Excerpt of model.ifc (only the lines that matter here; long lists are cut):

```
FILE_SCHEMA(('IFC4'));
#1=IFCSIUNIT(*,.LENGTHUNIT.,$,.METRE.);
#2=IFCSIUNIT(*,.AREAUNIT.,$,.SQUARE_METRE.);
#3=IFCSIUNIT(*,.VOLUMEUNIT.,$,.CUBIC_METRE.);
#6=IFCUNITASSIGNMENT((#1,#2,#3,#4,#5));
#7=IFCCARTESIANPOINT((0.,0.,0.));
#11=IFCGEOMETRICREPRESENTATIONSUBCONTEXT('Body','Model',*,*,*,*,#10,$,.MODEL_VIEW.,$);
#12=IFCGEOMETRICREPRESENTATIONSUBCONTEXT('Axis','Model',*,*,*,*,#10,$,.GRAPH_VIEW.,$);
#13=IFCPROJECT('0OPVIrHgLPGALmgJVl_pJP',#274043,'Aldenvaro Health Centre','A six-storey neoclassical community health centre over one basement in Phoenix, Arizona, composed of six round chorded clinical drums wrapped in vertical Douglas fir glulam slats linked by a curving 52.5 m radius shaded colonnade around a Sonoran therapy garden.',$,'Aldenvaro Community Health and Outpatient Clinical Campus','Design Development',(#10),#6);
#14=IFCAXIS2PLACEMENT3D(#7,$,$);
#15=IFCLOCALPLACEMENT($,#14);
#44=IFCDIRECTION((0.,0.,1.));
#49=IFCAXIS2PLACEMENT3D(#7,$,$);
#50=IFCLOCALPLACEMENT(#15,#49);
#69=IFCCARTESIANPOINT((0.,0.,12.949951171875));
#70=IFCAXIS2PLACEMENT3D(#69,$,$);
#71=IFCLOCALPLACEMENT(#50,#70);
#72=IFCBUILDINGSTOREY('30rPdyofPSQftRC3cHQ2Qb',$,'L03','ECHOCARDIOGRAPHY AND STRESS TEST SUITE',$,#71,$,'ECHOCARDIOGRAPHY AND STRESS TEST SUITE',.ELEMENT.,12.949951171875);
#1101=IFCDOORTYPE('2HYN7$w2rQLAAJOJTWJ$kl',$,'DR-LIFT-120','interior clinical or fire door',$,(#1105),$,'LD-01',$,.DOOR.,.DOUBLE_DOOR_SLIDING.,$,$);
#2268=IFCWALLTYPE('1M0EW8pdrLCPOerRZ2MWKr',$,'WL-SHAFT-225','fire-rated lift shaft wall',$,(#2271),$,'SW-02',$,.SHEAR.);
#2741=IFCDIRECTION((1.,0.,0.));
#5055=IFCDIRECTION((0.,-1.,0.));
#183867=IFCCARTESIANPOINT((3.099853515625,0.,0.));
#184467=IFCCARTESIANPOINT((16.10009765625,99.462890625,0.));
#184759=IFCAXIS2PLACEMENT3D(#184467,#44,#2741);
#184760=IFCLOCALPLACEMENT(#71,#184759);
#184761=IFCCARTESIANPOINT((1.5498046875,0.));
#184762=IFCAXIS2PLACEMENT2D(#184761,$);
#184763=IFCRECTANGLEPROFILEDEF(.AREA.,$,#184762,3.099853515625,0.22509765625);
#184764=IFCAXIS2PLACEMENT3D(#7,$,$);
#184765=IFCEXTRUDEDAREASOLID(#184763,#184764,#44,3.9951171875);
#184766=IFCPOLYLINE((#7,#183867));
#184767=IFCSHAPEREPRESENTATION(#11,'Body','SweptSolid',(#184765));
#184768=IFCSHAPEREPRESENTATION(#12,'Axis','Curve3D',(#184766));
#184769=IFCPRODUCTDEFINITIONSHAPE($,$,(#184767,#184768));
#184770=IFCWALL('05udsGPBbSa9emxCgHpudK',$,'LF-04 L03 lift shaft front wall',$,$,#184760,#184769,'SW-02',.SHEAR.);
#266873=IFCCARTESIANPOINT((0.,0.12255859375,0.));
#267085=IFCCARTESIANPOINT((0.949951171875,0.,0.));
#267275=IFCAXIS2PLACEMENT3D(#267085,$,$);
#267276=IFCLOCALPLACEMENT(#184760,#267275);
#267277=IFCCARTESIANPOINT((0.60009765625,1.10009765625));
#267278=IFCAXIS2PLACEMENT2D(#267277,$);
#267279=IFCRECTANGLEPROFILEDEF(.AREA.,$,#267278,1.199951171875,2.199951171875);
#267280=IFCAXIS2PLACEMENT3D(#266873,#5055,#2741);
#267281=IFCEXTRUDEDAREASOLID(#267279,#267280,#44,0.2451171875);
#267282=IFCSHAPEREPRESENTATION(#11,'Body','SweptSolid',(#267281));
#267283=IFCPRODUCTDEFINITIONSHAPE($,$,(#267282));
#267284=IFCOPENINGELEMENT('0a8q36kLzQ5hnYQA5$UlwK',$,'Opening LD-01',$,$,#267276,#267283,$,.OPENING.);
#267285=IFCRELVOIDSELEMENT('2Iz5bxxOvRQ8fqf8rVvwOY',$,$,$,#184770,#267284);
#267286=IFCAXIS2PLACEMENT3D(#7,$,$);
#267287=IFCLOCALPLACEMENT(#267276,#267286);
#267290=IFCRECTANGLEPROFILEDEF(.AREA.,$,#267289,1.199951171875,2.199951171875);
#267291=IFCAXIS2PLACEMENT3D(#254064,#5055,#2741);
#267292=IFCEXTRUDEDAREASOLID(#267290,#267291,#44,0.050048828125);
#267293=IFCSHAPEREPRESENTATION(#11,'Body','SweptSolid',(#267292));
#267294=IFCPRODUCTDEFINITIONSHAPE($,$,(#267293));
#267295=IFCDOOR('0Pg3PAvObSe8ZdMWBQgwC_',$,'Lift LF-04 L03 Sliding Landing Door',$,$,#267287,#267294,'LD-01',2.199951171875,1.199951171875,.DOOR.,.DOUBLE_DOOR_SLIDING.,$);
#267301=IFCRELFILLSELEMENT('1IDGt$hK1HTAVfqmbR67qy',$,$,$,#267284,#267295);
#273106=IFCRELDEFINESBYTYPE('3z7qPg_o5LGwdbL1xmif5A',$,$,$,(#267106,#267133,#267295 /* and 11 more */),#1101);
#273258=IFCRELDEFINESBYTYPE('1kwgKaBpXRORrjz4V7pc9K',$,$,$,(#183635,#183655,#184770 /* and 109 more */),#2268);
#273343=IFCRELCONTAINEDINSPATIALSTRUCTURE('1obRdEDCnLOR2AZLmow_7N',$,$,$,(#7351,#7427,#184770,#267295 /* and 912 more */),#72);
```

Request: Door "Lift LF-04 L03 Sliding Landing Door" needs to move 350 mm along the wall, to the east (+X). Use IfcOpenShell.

```python
import ifcopenshell
import ifcopenshell.api.geometry
import ifcopenshell.util.placement
import ifcopenshell.util.unit

model = ifcopenshell.open("model.ifc")
unit_scale = ifcopenshell.util.unit.calculate_unit_scale(model)

door = model.by_guid("0Pg3PAvObSe8ZdMWBQgwC_")
opening = door.FillsVoids[0].RelatingOpeningElement
wall = opening.VoidsElements[0].RelatingBuildingElement

wall_matrix = ifcopenshell.util.placement.get_local_placement(wall.ObjectPlacement)
shift = wall_matrix[:3, 0] * 0.35 / unit_scale
before = ifcopenshell.util.placement.get_local_placement(door.ObjectPlacement)[:3, 3].copy()

# The door is placed relative to its opening, so it follows when the opening moves.
matrix = ifcopenshell.util.placement.get_local_placement(opening.ObjectPlacement)
matrix[:3, 3] += shift
ifcopenshell.api.geometry.edit_object_placement(
    model, product=opening, matrix=matrix, is_si=False, should_transform_children=True
)

after = ifcopenshell.util.placement.get_local_placement(door.ObjectPlacement)[:3, 3]
print("door moved by", (after - before).round(3) + 0.0)

model.write("model_rev.ifc")
```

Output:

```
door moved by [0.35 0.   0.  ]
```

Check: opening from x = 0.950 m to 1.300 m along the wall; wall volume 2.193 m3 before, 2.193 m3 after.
